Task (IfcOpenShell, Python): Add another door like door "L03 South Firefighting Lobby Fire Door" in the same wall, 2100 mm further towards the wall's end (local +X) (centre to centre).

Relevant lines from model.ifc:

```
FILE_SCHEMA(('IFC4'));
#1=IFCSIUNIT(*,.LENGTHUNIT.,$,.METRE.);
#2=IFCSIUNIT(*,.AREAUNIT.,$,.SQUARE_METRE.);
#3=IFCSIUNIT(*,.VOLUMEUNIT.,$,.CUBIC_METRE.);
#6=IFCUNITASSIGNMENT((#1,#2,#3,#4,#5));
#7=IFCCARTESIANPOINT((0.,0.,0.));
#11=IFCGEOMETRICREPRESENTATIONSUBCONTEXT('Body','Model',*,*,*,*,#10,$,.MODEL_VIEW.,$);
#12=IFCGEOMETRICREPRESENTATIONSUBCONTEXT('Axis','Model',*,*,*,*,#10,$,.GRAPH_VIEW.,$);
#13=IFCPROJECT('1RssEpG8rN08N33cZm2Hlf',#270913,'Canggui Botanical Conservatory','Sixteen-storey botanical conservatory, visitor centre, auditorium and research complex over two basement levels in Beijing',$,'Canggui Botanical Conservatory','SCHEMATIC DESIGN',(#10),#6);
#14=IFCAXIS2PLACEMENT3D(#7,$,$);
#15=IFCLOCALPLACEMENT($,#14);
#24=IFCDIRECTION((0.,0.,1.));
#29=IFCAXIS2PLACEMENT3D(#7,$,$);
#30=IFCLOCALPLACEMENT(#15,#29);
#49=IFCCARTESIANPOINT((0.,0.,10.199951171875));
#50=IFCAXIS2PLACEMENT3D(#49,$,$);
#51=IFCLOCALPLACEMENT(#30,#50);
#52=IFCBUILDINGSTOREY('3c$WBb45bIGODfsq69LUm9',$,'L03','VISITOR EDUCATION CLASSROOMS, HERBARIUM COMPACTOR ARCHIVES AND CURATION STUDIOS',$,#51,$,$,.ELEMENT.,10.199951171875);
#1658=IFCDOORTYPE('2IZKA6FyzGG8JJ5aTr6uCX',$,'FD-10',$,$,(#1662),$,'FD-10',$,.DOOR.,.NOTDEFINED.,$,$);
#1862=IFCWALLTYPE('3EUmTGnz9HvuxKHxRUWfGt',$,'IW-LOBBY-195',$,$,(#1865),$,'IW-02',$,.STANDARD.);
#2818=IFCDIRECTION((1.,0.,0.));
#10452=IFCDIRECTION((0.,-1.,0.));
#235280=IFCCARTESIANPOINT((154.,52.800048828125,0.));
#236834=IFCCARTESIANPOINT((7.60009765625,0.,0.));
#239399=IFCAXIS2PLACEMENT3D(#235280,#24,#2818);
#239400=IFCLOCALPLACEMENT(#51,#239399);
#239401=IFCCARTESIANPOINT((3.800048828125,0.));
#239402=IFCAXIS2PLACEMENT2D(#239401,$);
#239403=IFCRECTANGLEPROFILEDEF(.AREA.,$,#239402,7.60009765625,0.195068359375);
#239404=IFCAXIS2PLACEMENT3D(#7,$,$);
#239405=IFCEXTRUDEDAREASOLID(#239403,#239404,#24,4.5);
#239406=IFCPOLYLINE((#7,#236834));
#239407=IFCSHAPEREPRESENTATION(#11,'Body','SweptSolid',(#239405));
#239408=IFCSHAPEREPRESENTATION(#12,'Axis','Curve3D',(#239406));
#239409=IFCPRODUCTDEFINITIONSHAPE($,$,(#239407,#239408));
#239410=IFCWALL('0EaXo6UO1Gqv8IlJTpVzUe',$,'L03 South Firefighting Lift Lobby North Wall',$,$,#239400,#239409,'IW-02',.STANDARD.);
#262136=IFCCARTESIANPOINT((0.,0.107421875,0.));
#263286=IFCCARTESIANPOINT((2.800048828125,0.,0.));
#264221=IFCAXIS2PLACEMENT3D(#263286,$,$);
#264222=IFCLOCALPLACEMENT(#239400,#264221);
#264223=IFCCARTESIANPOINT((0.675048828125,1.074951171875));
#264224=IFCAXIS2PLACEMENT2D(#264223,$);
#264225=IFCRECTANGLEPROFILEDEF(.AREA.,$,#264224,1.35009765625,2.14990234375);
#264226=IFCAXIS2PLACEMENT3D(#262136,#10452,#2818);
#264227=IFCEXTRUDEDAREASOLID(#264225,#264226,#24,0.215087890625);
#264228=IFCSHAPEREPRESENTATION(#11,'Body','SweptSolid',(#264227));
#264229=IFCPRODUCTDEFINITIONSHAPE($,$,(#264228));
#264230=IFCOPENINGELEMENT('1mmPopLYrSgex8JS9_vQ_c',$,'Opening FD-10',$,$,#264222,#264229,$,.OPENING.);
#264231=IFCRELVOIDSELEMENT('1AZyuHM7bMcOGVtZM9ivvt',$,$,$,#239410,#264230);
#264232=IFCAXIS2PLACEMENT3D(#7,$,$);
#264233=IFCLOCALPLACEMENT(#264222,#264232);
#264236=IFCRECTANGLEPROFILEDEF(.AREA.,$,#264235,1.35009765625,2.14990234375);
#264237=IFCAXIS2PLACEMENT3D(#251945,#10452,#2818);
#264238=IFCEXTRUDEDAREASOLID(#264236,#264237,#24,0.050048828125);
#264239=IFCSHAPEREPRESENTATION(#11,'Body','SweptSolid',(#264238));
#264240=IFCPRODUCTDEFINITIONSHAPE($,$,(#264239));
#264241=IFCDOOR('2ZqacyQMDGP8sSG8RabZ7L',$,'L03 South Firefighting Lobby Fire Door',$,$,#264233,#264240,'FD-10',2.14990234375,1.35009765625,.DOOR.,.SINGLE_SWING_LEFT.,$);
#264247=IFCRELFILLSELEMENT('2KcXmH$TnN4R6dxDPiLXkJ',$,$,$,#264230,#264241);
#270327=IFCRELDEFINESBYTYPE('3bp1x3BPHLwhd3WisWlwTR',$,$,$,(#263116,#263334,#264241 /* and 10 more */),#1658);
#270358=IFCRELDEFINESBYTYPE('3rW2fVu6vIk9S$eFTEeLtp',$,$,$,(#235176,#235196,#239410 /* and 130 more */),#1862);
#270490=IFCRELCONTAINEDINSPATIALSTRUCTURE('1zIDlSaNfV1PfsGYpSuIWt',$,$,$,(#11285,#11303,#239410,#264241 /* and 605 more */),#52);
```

```python
import ifcopenshell
import ifcopenshell.api.feature
import ifcopenshell.api.geometry
import ifcopenshell.api.root
import ifcopenshell.geom
import ifcopenshell.util.element
import ifcopenshell.util.placement
import ifcopenshell.util.shape
import ifcopenshell.util.unit

model = ifcopenshell.open("model.ifc")
unit_scale = ifcopenshell.util.unit.calculate_unit_scale(model)
settings = ifcopenshell.geom.settings()


def volume(element):
    """Net volume in cubic metres, openings subtracted."""
    shape = ifcopenshell.geom.create_shape(settings, element)
    return ifcopenshell.util.shape.get_volume(shape.geometry)


door = model.by_id(264241)
opening = door.FillsVoids[0].RelatingOpeningElement
wall = opening.VoidsElements[0].RelatingBuildingElement
before = volume(wall)
shift = ifcopenshell.util.placement.get_local_placement(wall.ObjectPlacement)[:3, 0] * 2.1 / unit_scale

# copy_class copies the void relationship, type, container and properties, but no geometry.
new_opening = ifcopenshell.api.root.copy_class(model, product=opening)
new_opening.Representation = ifcopenshell.util.element.copy_deep(
    model, opening.Representation, exclude=["IfcGeometricRepresentationContext", "IfcRepresentationMap"]
)
new_door = ifcopenshell.api.root.copy_class(model, product=door)
new_door.Representation = ifcopenshell.util.element.copy_deep(
    model, door.Representation, exclude=["IfcGeometricRepresentationContext", "IfcRepresentationMap"]
)
new_door.Tag = None
ifcopenshell.api.feature.add_filling(model, opening=new_opening, element=new_door)

for old, new in ((opening, new_opening), (door, new_door)):
    matrix = ifcopenshell.util.placement.get_local_placement(old.ObjectPlacement)
    matrix[:3, 3] += shift
    ifcopenshell.api.geometry.edit_object_placement(model, product=new, matrix=matrix, is_si=False)

after = volume(wall)

print(f"wall volume {before:.3f} -> {after:.3f} m3")

model.write("model_edited.ifc")
```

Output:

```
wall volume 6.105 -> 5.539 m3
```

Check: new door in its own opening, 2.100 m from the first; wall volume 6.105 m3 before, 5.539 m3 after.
